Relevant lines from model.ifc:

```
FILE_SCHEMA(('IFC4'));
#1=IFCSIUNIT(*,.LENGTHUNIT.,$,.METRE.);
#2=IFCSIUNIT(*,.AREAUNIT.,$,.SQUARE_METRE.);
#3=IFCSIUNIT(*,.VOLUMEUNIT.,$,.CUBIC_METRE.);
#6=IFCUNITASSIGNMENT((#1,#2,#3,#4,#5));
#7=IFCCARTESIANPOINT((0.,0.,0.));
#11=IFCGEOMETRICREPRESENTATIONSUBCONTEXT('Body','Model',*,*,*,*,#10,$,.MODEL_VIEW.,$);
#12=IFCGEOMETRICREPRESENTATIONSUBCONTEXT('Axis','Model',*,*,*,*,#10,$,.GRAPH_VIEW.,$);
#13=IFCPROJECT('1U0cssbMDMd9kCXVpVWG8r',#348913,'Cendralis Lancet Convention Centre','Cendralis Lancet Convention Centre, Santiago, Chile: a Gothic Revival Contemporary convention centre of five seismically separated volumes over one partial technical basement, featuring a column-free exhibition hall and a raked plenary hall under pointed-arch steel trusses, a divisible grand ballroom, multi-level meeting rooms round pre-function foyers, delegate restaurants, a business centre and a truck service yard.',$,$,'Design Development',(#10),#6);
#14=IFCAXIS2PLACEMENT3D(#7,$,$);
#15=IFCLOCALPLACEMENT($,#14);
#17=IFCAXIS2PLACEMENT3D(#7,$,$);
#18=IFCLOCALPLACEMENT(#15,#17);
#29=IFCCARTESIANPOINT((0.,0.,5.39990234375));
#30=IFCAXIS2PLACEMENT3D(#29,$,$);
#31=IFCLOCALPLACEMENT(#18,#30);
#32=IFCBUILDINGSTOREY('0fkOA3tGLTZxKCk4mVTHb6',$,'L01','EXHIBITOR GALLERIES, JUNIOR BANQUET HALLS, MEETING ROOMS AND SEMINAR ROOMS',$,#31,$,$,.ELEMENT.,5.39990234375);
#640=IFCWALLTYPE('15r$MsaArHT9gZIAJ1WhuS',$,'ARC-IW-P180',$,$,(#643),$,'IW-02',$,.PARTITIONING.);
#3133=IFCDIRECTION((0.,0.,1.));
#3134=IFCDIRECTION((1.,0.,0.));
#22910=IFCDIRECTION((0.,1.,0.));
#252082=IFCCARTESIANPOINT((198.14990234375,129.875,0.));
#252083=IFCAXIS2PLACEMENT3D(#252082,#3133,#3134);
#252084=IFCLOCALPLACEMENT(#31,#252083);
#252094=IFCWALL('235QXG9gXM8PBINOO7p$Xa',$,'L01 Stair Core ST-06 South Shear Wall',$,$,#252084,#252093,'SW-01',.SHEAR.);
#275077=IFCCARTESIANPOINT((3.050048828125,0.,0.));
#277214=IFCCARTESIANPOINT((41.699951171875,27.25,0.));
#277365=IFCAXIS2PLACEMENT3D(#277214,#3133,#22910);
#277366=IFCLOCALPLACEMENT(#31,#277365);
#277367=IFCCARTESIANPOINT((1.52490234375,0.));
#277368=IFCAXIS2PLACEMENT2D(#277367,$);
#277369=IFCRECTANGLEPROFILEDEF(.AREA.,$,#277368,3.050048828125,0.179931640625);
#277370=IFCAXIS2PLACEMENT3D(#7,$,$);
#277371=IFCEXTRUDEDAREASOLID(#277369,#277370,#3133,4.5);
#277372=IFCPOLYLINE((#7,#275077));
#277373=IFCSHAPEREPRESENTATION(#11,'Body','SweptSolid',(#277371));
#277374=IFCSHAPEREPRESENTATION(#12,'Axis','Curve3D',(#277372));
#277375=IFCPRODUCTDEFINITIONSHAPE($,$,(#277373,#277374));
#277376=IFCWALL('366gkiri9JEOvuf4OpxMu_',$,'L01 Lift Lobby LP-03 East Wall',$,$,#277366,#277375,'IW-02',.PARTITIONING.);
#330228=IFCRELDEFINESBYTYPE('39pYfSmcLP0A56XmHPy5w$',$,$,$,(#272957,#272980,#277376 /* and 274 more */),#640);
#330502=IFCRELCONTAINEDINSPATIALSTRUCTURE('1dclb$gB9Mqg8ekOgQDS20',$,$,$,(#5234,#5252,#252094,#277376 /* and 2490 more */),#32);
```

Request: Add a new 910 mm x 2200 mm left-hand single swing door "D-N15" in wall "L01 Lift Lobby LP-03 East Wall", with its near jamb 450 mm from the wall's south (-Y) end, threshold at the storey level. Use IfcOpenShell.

```python
import numpy as np
import ifcopenshell
import ifcopenshell.api.feature
import ifcopenshell.api.geometry
import ifcopenshell.api.root
import ifcopenshell.api.spatial
import ifcopenshell.geom
import ifcopenshell.util.element
import ifcopenshell.util.placement
import ifcopenshell.util.representation
import ifcopenshell.util.shape
import ifcopenshell.util.unit

model = ifcopenshell.open("model.ifc")
unit_scale = ifcopenshell.util.unit.calculate_unit_scale(model)
settings = ifcopenshell.geom.settings()


def volume(element):
    """Net volume in cubic metres, openings subtracted."""
    shape = ifcopenshell.geom.create_shape(settings, element)
    return ifcopenshell.util.shape.get_volume(shape.geometry)


wall = model.by_guid("366gkiri9JEOvuf4OpxMu_")
storey = ifcopenshell.util.element.get_container(wall, ifc_class="IfcBuildingStorey")
context = ifcopenshell.util.representation.get_context(model, "Model", "Body", "MODEL_VIEW")
before = volume(wall)

width, height, from_end, sill = 0.91, 2.2, 0.45, 0.0  # metres

# The wall runs along its own X axis, and the end named is its -X end.
wall_shape = ifcopenshell.geom.create_shape(settings, wall)
x, y, z = ifcopenshell.util.shape.get_vertices(wall_shape.geometry).T
start = x.min() + from_end
face, thickness = float(y.min()), float(y.max() - y.min())
wall_matrix = ifcopenshell.util.placement.get_local_placement(wall.ObjectPlacement)
level = ifcopenshell.util.placement.get_local_placement(storey.ObjectPlacement)[2, 3]


def in_wall(x, y):
    """Placement at x, y metres in the wall's axes, at sill height."""
    matrix = wall_matrix.copy()
    matrix[:, 3] = wall_matrix @ np.array([x / unit_scale, y / unit_scale, 0.0, 1.0])
    matrix[2, 3] = level + sill / unit_scale
    return matrix


# Opening: a box that overshoots both wall faces by 50 mm.
opening = ifcopenshell.api.root.create_entity(model, ifc_class="IfcOpeningElement", predefined_type="OPENING")
box = ifcopenshell.api.geometry.add_wall_representation(
    model, context=context, length=width, height=height, thickness=thickness + 0.1
)
ifcopenshell.api.geometry.assign_representation(model, product=opening, representation=box)
ifcopenshell.api.geometry.edit_object_placement(model, product=opening, matrix=in_wall(start, face - 0.05), is_si=False)
ifcopenshell.api.feature.add_feature(model, feature=opening, element=wall)

door = ifcopenshell.api.root.create_entity(model, ifc_class="IfcDoor", name="D-N15", predefined_type="DOOR")
door.OverallWidth, door.OverallHeight = width / unit_scale, height / unit_scale
door.OperationType = "SINGLE_SWING_LEFT"
body = ifcopenshell.api.geometry.add_door_representation(
    model,
    context=context,
    overall_width=door.OverallWidth,
    overall_height=door.OverallHeight,
    operation_type="SINGLE_SWING_LEFT",
    lining_properties={"LiningDepth": thickness / unit_scale, "ThresholdDepth": thickness / unit_scale},
)
ifcopenshell.api.geometry.assign_representation(model, product=door, representation=body)
ifcopenshell.api.spatial.assign_container(model, products=[door], relating_structure=storey)
ifcopenshell.api.feature.add_filling(model, opening=opening, element=door)

# The lining spans the wall, so the door starts at the wall face.
ifcopenshell.api.geometry.edit_object_placement(model, product=door, matrix=in_wall(start, face), is_si=False)

after = volume(wall)

print(f"wall volume {before:.3f} -> {after:.3f} m3")

model.write("model_v2.ifc")
```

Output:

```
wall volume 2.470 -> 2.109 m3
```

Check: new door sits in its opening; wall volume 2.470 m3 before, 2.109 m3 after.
